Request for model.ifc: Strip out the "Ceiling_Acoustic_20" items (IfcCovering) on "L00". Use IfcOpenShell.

First a look at what the model holds.

```python
import ifcopenshell
import ifcopenshell.util.element

model = ifcopenshell.open("model.ifc")
print(model.schema)
storey = next(s for s in model.by_type("IfcBuildingStorey") if s.Name == "L00")
coverings = [e for e in ifcopenshell.util.element.get_decomposition(storey) if e.is_a("IfcCovering")]
seen = {}
for e in coverings:
    element_type = ifcopenshell.util.element.get_type(e)
    name = element_type.Name if element_type not in (None, e) else None
    seen[name] = seen.get(name, 0) + 1
for name, count in sorted(seen.items(), key=str):
    print(count, "x", name)
```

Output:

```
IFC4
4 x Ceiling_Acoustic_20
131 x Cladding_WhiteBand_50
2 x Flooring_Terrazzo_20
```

```python
import ifcopenshell
import ifcopenshell.api.root
import ifcopenshell.util.element

model = ifcopenshell.open("model.ifc")

storey = next(s for s in model.by_type("IfcBuildingStorey") if s.Name == "L00")
coverings = [e for e in ifcopenshell.util.element.get_decomposition(storey) if e.is_a("IfcCovering")]
targets = [e for e in coverings if (t := ifcopenshell.util.element.get_type(e)) not in (None, e) and t.Name == "Ceiling_Acoustic_20"]

for e in targets:
    ifcopenshell.api.root.remove_product(model, product=e)
print(len(targets), "removed")

model.write("model-out.ifc")
```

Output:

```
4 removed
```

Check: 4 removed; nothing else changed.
